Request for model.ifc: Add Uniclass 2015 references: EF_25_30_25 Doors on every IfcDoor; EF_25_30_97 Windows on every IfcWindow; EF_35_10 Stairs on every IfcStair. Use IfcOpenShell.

First a look at what the model holds.

```python
import ifcopenshell

model = ifcopenshell.open("model.ifc")
print(model.schema)
print("classifications:", [c.Name for c in model.by_type("IfcClassification")])
for ifc_class in ("IfcDoor", "IfcRoof", "IfcStair", "IfcWall", "IfcWindow"):
    print(ifc_class, len(model.by_type(ifc_class)))
```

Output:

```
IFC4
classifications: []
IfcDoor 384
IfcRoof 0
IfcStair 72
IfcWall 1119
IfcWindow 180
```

```python
import ifcopenshell
import ifcopenshell.api.classification

model = ifcopenshell.open("model.ifc")

system = ifcopenshell.api.classification.add_classification(model, classification="Uniclass 2015")

codes = {
    "IfcDoor": ("EF_25_30_25", "Doors"),
    "IfcWindow": ("EF_25_30_97", "Windows"),
    "IfcStair": ("EF_35_10", "Stairs"),
}
for ifc_class, (code, name) in codes.items():
    products = model.by_type(ifc_class)
    ifcopenshell.api.classification.add_reference(
        model, products=products, classification=system, identification=code, name=name
    )
    print(code, len(products))

model.write("model-out.ifc")
```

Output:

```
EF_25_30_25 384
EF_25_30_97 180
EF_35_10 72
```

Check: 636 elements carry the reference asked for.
